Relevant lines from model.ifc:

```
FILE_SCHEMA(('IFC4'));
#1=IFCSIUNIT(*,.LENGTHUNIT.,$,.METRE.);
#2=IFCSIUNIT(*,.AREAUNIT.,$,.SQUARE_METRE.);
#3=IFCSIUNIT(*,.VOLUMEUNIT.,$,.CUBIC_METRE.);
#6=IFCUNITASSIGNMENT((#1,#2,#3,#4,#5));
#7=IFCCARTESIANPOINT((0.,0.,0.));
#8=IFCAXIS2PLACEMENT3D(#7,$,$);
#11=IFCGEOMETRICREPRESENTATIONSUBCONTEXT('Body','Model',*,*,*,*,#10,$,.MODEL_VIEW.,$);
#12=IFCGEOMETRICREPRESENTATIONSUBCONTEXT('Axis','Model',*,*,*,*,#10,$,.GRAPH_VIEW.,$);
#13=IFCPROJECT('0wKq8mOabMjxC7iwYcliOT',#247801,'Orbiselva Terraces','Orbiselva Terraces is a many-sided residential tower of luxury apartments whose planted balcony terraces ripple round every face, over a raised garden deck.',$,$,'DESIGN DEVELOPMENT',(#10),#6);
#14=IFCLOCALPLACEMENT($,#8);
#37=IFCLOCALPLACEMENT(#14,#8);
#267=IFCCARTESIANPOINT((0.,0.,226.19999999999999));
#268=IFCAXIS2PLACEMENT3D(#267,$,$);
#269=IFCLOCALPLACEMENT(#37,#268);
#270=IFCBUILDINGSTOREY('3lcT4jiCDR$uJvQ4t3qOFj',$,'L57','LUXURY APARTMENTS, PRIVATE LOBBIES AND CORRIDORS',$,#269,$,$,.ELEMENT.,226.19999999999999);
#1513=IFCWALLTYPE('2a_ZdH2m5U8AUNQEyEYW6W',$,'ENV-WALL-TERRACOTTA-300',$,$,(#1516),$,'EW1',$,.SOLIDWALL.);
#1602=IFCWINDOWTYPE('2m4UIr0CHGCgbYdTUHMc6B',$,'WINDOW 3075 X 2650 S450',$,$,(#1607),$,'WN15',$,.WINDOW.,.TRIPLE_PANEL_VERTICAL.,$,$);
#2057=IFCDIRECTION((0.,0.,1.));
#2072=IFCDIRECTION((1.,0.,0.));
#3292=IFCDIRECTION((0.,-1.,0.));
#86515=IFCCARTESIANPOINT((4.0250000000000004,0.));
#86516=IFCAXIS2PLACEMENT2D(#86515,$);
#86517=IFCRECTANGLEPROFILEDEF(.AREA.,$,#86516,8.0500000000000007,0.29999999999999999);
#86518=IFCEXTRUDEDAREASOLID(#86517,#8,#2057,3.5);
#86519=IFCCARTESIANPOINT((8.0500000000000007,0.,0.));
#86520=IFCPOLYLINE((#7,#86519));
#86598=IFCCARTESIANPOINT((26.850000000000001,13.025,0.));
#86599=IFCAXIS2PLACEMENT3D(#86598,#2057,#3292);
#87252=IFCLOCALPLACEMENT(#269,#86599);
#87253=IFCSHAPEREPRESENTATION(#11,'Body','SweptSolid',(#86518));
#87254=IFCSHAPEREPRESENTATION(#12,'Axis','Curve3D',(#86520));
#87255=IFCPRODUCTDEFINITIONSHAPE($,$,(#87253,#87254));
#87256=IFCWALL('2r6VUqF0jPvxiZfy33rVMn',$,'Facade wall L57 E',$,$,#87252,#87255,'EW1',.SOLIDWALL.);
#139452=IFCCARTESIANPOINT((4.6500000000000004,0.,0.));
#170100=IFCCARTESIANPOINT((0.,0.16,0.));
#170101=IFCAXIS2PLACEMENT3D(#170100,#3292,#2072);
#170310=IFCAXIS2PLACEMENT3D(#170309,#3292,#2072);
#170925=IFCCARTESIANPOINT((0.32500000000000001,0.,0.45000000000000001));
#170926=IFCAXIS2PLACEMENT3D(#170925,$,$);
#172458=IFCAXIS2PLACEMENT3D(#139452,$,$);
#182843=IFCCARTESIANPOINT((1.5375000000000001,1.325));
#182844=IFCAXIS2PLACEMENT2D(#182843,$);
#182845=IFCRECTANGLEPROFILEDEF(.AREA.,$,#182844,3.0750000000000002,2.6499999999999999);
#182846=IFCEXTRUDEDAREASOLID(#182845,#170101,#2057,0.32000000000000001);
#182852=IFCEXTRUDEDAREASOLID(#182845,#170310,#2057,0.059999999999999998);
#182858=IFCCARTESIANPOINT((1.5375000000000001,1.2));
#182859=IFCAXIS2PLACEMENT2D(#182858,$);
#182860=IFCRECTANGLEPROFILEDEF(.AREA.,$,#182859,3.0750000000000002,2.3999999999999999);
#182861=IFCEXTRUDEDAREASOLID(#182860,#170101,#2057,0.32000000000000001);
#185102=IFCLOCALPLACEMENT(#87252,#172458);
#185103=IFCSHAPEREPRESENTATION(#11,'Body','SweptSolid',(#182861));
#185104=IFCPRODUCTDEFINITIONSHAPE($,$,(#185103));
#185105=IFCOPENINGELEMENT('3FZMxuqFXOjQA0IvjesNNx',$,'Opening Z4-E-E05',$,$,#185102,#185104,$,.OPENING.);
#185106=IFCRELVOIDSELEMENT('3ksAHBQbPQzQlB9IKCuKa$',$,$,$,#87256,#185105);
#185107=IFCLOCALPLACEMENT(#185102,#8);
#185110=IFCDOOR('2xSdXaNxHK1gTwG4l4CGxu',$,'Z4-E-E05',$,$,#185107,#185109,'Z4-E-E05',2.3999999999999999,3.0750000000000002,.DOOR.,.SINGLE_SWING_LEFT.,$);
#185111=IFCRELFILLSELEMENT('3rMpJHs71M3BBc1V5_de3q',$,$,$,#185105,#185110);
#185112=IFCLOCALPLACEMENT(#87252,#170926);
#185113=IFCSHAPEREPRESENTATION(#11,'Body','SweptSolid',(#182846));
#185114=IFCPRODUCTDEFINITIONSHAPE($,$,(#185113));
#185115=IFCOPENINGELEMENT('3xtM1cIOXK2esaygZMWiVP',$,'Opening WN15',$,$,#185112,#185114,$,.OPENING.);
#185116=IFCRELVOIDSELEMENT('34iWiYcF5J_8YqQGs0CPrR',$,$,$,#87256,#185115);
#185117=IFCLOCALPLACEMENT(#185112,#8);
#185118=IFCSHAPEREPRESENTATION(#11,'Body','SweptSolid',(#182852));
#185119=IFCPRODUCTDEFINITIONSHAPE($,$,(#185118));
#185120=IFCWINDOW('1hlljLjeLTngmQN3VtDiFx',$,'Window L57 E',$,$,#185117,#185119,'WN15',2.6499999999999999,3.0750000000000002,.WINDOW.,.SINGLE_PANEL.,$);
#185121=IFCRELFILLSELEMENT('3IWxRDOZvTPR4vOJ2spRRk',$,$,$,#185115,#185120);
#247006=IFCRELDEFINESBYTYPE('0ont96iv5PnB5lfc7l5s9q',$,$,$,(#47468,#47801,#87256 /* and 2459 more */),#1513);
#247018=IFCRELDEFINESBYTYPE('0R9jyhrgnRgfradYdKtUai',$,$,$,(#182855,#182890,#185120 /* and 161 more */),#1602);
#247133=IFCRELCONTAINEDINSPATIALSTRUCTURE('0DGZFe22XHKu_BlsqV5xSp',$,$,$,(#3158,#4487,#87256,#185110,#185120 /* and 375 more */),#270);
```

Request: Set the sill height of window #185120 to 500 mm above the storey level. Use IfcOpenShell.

```python
import numpy as np
import ifcopenshell
import ifcopenshell.api.geometry
import ifcopenshell.geom
import ifcopenshell.util.element
import ifcopenshell.util.placement
import ifcopenshell.util.shape
import ifcopenshell.util.unit

model = ifcopenshell.open("model.ifc")
unit_scale = ifcopenshell.util.unit.calculate_unit_scale(model)

window = model.by_id(185120)
opening = window.FillsVoids[0].RelatingOpeningElement
storey = ifcopenshell.util.element.get_container(window, ifc_class="IfcBuildingStorey")
level = ifcopenshell.util.placement.get_local_placement(storey.ObjectPlacement)[2, 3]

# The opening's origin need not be at the sill, so measure its lowest point.
shape = ifcopenshell.geom.create_shape(ifcopenshell.geom.settings(), opening)
bottom = ifcopenshell.util.shape.get_shape_bottom_elevation(shape, shape.geometry) / unit_scale
dz = level + 0.5 / unit_scale - bottom

shift = np.array([0.0, 0.0, dz])
# The window is placed relative to its opening, so it follows when the opening moves.
matrix = ifcopenshell.util.placement.get_local_placement(opening.ObjectPlacement)
matrix[:3, 3] += shift
ifcopenshell.api.geometry.edit_object_placement(
    model, product=opening, matrix=matrix, is_si=False, should_transform_children=True
)

print(f"moved by {dz * unit_scale:+.3f} m")

model.write("model_updated.ifc")
```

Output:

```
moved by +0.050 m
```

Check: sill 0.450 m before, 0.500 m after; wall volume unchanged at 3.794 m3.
